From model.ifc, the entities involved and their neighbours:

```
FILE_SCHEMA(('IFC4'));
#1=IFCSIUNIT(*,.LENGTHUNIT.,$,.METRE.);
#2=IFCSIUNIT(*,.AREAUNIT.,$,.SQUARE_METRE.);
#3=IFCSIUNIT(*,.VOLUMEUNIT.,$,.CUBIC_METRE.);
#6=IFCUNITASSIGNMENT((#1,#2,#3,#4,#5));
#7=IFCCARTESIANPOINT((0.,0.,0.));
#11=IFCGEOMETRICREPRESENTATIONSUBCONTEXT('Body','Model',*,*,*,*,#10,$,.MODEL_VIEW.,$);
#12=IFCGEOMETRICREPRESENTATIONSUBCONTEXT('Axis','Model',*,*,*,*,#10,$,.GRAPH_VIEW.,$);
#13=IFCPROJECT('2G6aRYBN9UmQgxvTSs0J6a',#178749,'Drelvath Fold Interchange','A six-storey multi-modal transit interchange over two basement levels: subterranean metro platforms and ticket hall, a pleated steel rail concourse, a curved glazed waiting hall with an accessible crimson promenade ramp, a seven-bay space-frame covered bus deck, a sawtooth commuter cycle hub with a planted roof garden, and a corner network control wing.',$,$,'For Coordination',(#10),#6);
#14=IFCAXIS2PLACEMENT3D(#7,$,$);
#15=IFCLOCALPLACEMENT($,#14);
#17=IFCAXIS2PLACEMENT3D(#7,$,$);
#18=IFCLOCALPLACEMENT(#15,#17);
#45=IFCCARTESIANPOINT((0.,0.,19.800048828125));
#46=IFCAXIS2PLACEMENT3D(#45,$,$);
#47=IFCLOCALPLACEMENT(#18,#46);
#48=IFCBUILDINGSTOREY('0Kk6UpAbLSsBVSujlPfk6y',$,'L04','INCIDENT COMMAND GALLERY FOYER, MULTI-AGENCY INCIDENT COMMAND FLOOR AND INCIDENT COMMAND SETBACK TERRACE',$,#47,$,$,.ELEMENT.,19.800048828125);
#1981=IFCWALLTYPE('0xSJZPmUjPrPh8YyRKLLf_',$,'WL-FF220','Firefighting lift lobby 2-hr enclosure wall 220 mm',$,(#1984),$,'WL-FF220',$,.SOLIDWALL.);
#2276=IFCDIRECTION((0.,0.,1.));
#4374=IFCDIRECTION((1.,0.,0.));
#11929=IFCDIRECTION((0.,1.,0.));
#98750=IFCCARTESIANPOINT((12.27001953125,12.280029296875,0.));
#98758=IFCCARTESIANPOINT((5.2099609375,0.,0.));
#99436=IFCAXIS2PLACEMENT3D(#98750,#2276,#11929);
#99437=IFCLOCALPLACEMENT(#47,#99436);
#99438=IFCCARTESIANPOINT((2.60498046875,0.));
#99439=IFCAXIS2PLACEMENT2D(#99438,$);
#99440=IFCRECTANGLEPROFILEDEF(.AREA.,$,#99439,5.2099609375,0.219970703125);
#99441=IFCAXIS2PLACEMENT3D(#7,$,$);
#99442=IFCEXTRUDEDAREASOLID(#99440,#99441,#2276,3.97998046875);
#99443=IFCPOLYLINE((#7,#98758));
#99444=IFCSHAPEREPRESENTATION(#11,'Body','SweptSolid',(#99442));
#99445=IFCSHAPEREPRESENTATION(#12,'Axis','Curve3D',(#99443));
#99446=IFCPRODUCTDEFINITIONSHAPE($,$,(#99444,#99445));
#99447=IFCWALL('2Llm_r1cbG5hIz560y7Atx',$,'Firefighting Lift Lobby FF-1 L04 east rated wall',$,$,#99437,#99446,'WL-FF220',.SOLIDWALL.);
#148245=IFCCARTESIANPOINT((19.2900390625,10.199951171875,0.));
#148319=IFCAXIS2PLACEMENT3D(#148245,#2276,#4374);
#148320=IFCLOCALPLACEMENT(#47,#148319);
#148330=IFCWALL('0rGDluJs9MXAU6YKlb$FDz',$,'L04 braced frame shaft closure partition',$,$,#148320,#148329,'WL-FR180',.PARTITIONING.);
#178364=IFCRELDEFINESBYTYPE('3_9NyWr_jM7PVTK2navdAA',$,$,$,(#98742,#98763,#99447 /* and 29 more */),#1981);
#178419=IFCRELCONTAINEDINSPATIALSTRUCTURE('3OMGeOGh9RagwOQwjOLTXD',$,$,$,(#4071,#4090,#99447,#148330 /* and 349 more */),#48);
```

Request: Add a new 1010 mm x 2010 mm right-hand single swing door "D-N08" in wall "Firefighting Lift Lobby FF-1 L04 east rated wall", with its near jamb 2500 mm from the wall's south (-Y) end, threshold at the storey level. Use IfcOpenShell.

```python
import numpy as np
import ifcopenshell
import ifcopenshell.api.feature
import ifcopenshell.api.geometry
import ifcopenshell.api.root
import ifcopenshell.api.spatial
import ifcopenshell.geom
import ifcopenshell.util.element
import ifcopenshell.util.placement
import ifcopenshell.util.representation
import ifcopenshell.util.shape
import ifcopenshell.util.unit

model = ifcopenshell.open("model.ifc")
unit_scale = ifcopenshell.util.unit.calculate_unit_scale(model)
settings = ifcopenshell.geom.settings()


def volume(element):
    """Net volume in cubic metres, openings subtracted."""
    shape = ifcopenshell.geom.create_shape(settings, element)
    return ifcopenshell.util.shape.get_volume(shape.geometry)


wall = model.by_guid("2Llm_r1cbG5hIz560y7Atx")
storey = ifcopenshell.util.element.get_container(wall, ifc_class="IfcBuildingStorey")
context = ifcopenshell.util.representation.get_context(model, "Model", "Body", "MODEL_VIEW")
before = volume(wall)

width, height, from_end, sill = 1.01, 2.01, 2.5, 0.0  # metres

# The wall runs along its own X axis, and the end named is its -X end.
wall_shape = ifcopenshell.geom.create_shape(settings, wall)
x, y, z = ifcopenshell.util.shape.get_vertices(wall_shape.geometry).T
start = x.min() + from_end
face, thickness = float(y.min()), float(y.max() - y.min())
wall_matrix = ifcopenshell.util.placement.get_local_placement(wall.ObjectPlacement)
level = ifcopenshell.util.placement.get_local_placement(storey.ObjectPlacement)[2, 3]


def in_wall(x, y):
    """Placement at x, y metres in the wall's axes, at sill height."""
    matrix = wall_matrix.copy()
    matrix[:, 3] = wall_matrix @ np.array([x / unit_scale, y / unit_scale, 0.0, 1.0])
    matrix[2, 3] = level + sill / unit_scale
    return matrix


# Opening: a box that overshoots both wall faces by 50 mm.
opening = ifcopenshell.api.root.create_entity(model, ifc_class="IfcOpeningElement", predefined_type="OPENING")
box = ifcopenshell.api.geometry.add_wall_representation(
    model, context=context, length=width, height=height, thickness=thickness + 0.1
)
ifcopenshell.api.geometry.assign_representation(model, product=opening, representation=box)
ifcopenshell.api.geometry.edit_object_placement(model, product=opening, matrix=in_wall(start, face - 0.05), is_si=False)
ifcopenshell.api.feature.add_feature(model, feature=opening, element=wall)

door = ifcopenshell.api.root.create_entity(model, ifc_class="IfcDoor", name="D-N08", predefined_type="DOOR")
door.OverallWidth, door.OverallHeight = width / unit_scale, height / unit_scale
door.OperationType = "SINGLE_SWING_RIGHT"
body = ifcopenshell.api.geometry.add_door_representation(
    model,
    context=context,
    overall_width=door.OverallWidth,
    overall_height=door.OverallHeight,
    operation_type="SINGLE_SWING_RIGHT",
    lining_properties={"LiningDepth": thickness / unit_scale, "ThresholdDepth": thickness / unit_scale},
)
ifcopenshell.api.geometry.assign_representation(model, product=door, representation=body)
ifcopenshell.api.spatial.assign_container(model, products=[door], relating_structure=storey)
ifcopenshell.api.feature.add_filling(model, opening=opening, element=door)

# The lining spans the wall, so the door starts at the wall face.
ifcopenshell.api.geometry.edit_object_placement(model, product=door, matrix=in_wall(start, face), is_si=False)

after = volume(wall)

print(f"wall volume {before:.3f} -> {after:.3f} m3")

model.write("model-out.ifc")
```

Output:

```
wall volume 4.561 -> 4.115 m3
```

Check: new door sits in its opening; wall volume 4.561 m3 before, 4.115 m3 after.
